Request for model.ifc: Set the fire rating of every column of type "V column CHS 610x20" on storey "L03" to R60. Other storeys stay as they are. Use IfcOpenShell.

First a look at what the model holds.

```python
import ifcopenshell
import ifcopenshell.util.element

model = ifcopenshell.open("model.ifc")
print(model.schema)
storey = next(s for s in model.by_type("IfcBuildingStorey") if s.Name == "L03")
columns = [e for e in ifcopenshell.util.element.get_decomposition(storey) if e.is_a("IfcColumn")]
seen = {}
for e in columns:
    element_type = ifcopenshell.util.element.get_type(e)
    key = (element_type.Name if element_type != e and element_type else None, ifcopenshell.util.element.get_pset(e, "Pset_ColumnCommon", "FireRating"))
    seen[key] = seen.get(key, 0) + 1
for (name, value), count in sorted(seen.items(), key=str):
    print(count, "x", name, "|", value)
```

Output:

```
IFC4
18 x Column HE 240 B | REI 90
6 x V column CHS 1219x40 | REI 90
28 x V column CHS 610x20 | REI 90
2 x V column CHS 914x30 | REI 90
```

```python
import ifcopenshell
import ifcopenshell.api.pset
import ifcopenshell.util.element

model = ifcopenshell.open("model.ifc")

storey = next(s for s in model.by_type("IfcBuildingStorey") if s.Name == "L03")
columns = [e for e in ifcopenshell.util.element.get_decomposition(storey) if e.is_a("IfcColumn")]

count = 0
for e in columns:
    element_type = ifcopenshell.util.element.get_type(e)
    if element_type in (None, e) or element_type.Name != "V column CHS 610x20":
        continue
    # add_pset returns the element's existing set when there is one.
    pset = ifcopenshell.api.pset.add_pset(model, product=e, name="Pset_ColumnCommon")
    ifcopenshell.api.pset.edit_pset(model, pset=pset, properties={"FireRating": "R60"})
    count += 1

print(count, "columns updated")

model.write("model_rev.ifc")
```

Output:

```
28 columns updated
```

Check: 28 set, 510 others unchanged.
